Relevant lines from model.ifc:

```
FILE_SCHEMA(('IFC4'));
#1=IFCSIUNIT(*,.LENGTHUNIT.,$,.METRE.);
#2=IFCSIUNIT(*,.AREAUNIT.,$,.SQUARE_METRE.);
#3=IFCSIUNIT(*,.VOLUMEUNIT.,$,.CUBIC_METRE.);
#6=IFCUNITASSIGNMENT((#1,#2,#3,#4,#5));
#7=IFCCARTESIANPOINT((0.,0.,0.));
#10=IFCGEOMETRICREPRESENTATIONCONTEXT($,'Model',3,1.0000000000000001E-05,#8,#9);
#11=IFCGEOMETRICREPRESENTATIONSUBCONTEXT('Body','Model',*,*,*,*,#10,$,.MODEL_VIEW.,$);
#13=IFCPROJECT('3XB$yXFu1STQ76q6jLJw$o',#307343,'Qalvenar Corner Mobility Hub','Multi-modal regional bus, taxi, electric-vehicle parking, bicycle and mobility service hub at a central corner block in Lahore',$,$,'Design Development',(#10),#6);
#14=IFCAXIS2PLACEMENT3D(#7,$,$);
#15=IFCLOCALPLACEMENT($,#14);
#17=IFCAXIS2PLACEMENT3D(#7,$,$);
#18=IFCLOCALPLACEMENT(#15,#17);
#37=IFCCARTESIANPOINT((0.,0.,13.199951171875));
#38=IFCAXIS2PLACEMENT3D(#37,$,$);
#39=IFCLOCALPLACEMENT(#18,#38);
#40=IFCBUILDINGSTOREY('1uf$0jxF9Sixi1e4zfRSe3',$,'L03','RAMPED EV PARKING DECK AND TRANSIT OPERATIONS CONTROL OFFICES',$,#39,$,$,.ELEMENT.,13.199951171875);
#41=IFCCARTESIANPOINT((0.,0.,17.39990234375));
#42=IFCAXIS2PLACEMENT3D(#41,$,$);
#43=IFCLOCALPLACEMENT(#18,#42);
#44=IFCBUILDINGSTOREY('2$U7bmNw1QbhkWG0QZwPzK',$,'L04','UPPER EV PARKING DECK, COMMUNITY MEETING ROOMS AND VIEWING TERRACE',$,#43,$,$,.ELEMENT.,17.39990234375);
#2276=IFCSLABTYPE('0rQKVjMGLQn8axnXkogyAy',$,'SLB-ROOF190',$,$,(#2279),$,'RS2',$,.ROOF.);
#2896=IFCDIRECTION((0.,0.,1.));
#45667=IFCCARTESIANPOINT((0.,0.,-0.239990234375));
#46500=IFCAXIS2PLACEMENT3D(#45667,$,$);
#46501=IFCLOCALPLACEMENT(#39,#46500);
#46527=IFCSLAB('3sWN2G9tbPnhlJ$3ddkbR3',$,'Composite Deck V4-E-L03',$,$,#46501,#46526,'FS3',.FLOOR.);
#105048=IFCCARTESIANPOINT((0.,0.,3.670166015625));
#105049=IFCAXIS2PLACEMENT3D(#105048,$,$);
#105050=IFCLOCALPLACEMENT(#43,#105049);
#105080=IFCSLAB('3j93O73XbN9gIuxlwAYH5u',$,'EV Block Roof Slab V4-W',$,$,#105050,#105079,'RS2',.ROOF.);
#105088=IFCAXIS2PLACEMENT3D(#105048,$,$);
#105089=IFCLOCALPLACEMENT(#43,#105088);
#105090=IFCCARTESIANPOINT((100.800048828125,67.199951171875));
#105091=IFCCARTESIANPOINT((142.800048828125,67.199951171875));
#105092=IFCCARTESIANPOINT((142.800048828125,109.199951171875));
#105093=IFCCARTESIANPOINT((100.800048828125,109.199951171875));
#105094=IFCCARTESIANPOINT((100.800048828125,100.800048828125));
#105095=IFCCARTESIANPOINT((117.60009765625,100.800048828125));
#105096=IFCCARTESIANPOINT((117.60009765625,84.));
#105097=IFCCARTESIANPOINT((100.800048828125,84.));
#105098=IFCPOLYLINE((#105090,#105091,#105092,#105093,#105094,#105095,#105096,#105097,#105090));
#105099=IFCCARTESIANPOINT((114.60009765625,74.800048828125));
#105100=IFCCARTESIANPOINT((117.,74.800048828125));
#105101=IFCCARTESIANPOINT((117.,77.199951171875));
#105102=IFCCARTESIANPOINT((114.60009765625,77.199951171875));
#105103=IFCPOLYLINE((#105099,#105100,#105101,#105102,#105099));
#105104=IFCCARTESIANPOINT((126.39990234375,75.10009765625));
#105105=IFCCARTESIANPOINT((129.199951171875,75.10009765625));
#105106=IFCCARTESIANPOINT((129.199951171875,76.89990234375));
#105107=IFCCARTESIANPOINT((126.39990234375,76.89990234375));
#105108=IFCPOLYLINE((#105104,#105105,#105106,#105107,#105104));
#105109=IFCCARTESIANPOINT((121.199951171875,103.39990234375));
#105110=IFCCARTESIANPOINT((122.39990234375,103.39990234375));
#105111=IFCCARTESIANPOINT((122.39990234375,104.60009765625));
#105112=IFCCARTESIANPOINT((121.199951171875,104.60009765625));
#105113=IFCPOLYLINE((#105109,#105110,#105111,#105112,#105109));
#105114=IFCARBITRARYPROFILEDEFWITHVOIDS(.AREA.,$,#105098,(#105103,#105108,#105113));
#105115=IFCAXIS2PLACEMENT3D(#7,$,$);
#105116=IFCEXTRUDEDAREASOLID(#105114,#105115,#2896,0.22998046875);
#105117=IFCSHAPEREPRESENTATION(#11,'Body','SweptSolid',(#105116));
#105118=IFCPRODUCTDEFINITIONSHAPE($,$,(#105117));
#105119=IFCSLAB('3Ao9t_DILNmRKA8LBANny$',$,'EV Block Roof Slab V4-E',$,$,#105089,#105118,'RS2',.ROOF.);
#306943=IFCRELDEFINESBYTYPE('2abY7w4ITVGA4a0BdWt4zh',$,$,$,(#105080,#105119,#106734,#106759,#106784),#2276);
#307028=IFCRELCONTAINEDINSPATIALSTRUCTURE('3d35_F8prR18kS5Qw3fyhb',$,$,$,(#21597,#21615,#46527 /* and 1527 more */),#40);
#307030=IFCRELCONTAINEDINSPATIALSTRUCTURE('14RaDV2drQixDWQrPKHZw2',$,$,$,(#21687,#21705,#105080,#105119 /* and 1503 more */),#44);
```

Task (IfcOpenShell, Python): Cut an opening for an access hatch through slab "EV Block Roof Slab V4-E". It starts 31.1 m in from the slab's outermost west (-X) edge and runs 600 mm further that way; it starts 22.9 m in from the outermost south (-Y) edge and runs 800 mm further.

```python
import numpy as np
import ifcopenshell
import ifcopenshell.api.feature
import ifcopenshell.api.geometry
import ifcopenshell.api.root
import ifcopenshell.geom
import ifcopenshell.util.placement
import ifcopenshell.util.representation
import ifcopenshell.util.shape
import ifcopenshell.util.unit

model = ifcopenshell.open("model.ifc")
unit_scale = ifcopenshell.util.unit.calculate_unit_scale(model)
settings = ifcopenshell.geom.settings()


def volume(element):
    """Net volume in cubic metres, openings subtracted."""
    shape = ifcopenshell.geom.create_shape(settings, element)
    return ifcopenshell.util.shape.get_volume(shape.geometry)


slab = model.by_guid("3Ao9t_DILNmRKA8LBANny$")
before = volume(slab)

# Extent in the slab's own axes, in metres. The edges named are its -X and -Y sides.
slab_shape = ifcopenshell.geom.create_shape(settings, slab)
vertices = ifcopenshell.util.shape.get_vertices(slab_shape.geometry)
x_min, y_min, bottom = vertices.min(axis=0)
top = vertices[:, 2].max()

opening = ifcopenshell.api.root.create_entity(model, ifc_class="IfcOpeningElement", name="Access hatch opening", predefined_type="OPENING")
context = ifcopenshell.util.representation.get_context(model, "Model", "Body", "MODEL_VIEW")
width, depth = 0.6, 0.8
outline = [(0.0, 0.0), (width, 0.0), (width, depth), (0.0, depth), (0.0, 0.0)]
# Overshoot both faces by 50 mm so the cut is clean.
shape = ifcopenshell.api.geometry.add_slab_representation(
    model, context=context, depth=top - bottom + 0.1, polyline=outline
)
ifcopenshell.api.geometry.assign_representation(model, product=opening, representation=shape)

matrix = ifcopenshell.util.placement.get_local_placement(slab.ObjectPlacement)
matrix[:, 3] = matrix @ np.append(np.array([x_min + 31.1, y_min + 22.9, bottom - 0.05]) / unit_scale, 1.0)
ifcopenshell.api.geometry.edit_object_placement(model, product=opening, matrix=matrix, is_si=False)
ifcopenshell.api.feature.add_feature(model, feature=opening, element=slab)

after = volume(slab)

print(f"slab volume {before:.3f} -> {after:.3f} m3")

model.write("model_rev.ifc")
```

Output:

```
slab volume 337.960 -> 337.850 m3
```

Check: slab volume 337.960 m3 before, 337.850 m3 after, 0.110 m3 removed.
